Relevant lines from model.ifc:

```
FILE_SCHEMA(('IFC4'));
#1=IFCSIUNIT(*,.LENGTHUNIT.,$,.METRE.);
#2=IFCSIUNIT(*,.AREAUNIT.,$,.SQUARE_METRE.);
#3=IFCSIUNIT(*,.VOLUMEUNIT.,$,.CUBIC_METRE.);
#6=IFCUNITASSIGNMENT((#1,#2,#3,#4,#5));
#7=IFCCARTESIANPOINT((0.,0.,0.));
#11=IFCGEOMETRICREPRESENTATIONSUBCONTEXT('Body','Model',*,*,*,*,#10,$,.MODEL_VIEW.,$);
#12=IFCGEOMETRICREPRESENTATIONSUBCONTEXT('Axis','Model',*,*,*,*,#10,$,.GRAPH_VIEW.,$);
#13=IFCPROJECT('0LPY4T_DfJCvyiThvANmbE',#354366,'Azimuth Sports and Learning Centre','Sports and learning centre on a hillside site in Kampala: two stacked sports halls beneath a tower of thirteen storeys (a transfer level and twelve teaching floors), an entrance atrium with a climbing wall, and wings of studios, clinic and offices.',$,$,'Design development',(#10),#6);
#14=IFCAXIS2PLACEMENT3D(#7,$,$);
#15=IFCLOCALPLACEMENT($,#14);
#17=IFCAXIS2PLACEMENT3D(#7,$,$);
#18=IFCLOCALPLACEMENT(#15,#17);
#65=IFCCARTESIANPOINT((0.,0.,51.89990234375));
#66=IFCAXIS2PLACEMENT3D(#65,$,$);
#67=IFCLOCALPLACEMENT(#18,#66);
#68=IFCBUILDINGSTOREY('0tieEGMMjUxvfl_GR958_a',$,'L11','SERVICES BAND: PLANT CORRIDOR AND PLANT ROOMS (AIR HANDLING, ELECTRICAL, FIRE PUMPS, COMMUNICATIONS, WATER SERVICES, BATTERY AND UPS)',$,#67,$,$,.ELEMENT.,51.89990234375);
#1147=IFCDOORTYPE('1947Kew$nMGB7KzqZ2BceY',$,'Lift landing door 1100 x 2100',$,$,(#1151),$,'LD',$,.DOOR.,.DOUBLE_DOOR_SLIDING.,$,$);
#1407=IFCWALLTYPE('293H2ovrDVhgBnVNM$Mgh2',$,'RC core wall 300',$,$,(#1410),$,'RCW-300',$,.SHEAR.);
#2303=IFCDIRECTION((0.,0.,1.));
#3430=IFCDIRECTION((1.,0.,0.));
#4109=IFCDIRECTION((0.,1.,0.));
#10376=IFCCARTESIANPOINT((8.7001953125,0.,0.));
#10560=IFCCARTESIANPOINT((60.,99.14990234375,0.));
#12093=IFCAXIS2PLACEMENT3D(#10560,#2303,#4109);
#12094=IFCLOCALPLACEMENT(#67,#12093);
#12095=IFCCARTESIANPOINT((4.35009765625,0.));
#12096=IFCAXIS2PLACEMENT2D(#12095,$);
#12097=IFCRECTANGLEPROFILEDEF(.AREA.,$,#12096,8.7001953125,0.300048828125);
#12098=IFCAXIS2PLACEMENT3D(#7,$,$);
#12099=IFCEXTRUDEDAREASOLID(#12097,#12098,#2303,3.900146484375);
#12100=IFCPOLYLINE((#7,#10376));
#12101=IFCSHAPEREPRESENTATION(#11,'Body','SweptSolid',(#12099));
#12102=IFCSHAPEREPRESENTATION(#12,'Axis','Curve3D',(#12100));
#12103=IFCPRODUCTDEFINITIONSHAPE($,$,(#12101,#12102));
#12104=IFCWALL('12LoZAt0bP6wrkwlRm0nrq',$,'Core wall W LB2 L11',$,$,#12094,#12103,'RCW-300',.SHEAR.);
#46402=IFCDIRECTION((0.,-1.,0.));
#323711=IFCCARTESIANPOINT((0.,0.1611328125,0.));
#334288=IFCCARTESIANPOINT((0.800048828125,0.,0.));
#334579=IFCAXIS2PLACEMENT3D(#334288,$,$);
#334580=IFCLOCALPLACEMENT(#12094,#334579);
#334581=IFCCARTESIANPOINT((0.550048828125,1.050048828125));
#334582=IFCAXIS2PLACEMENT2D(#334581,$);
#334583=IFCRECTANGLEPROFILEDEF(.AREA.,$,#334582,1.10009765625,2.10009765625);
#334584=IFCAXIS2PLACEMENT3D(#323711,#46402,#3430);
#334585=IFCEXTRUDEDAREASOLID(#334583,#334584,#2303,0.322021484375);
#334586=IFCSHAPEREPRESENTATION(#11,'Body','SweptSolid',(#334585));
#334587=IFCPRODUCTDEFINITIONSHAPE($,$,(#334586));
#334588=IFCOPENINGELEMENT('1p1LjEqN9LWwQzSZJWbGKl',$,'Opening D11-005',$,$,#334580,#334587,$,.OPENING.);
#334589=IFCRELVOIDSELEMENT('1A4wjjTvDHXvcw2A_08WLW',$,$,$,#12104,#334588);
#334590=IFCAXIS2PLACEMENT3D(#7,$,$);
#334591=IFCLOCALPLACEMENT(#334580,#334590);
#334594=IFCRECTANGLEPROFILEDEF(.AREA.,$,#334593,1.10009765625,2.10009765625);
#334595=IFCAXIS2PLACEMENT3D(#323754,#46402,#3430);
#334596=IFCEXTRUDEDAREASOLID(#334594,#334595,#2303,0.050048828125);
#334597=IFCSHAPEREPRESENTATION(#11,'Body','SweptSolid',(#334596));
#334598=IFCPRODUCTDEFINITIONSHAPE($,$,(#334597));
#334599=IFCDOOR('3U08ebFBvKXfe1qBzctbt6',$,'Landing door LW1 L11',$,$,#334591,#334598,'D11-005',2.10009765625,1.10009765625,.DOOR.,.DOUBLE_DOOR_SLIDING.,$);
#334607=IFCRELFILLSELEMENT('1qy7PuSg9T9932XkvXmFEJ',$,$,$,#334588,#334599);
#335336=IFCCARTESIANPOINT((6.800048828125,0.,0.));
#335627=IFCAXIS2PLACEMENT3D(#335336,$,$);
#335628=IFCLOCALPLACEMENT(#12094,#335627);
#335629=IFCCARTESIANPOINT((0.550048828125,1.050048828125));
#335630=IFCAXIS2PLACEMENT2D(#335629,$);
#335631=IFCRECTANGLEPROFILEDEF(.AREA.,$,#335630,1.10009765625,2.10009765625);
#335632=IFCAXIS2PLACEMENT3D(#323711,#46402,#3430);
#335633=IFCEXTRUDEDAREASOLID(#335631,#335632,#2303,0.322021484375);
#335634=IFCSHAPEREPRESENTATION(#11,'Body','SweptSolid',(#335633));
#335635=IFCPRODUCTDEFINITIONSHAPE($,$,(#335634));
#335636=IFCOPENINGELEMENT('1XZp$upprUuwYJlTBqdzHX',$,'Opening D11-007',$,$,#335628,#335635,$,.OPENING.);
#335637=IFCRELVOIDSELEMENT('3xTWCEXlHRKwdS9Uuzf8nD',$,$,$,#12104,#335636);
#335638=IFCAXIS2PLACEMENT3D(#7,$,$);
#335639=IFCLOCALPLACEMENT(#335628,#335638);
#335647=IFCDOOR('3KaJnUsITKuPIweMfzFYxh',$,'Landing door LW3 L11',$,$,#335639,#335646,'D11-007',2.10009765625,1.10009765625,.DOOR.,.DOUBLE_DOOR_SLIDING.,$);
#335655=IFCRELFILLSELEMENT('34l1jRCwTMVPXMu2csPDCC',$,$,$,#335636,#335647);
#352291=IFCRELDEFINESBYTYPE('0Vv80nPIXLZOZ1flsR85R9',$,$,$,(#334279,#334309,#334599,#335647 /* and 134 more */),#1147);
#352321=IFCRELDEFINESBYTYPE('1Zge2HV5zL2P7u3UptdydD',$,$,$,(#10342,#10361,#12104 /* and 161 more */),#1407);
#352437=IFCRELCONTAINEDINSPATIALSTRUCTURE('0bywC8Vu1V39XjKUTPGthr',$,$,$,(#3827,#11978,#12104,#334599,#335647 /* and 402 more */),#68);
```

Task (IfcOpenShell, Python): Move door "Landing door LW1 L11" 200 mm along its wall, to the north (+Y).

```python
import ifcopenshell
import ifcopenshell.api.geometry
import ifcopenshell.util.placement
import ifcopenshell.util.unit

model = ifcopenshell.open("model.ifc")
unit_scale = ifcopenshell.util.unit.calculate_unit_scale(model)

door = model.by_guid("3U08ebFBvKXfe1qBzctbt6")
opening = door.FillsVoids[0].RelatingOpeningElement
wall = opening.VoidsElements[0].RelatingBuildingElement

wall_matrix = ifcopenshell.util.placement.get_local_placement(wall.ObjectPlacement)
shift = wall_matrix[:3, 0] * 0.2 / unit_scale
before = ifcopenshell.util.placement.get_local_placement(door.ObjectPlacement)[:3, 3].copy()

# The door is placed relative to its opening, so it follows when the opening moves.
matrix = ifcopenshell.util.placement.get_local_placement(opening.ObjectPlacement)
matrix[:3, 3] += shift
ifcopenshell.api.geometry.edit_object_placement(
    model, product=opening, matrix=matrix, is_si=False, should_transform_children=True
)

after = ifcopenshell.util.placement.get_local_placement(door.ObjectPlacement)[:3, 3]
print("door moved by", (after - before).round(3) + 0.0)

model.write("model-out.ifc")
```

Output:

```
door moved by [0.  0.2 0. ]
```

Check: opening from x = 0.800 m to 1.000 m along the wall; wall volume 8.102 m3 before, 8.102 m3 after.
